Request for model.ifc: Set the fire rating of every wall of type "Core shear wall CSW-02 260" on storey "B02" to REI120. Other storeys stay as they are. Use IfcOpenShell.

First a look at what the model holds.

```python
import ifcopenshell
import ifcopenshell.util.element

model = ifcopenshell.open("model.ifc")
print(model.schema)
storey = next(s for s in model.by_type("IfcBuildingStorey") if s.Name == "B02")
walls = [e for e in ifcopenshell.util.element.get_decomposition(storey) if e.is_a("IfcWall")]
seen = {}
for e in walls:
    element_type = ifcopenshell.util.element.get_type(e)
    key = (element_type.Name if element_type != e and element_type else None, ifcopenshell.util.element.get_pset(e, "Pset_WallCommon", "FireRating"))
    seen[key] = seen.get(key, 0) + 1
for (name, value), count in sorted(seen.items(), key=str):
    print(count, "x", name, "|", value)
```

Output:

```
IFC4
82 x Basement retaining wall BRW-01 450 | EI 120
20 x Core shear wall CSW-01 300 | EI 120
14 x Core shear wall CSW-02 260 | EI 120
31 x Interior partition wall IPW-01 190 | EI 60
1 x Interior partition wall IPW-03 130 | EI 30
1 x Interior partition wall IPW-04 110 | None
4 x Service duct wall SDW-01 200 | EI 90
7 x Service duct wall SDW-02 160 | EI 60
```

```python
import ifcopenshell
import ifcopenshell.api.pset
import ifcopenshell.util.element

model = ifcopenshell.open("model.ifc")

storey = next(s for s in model.by_type("IfcBuildingStorey") if s.Name == "B02")
walls = [e for e in ifcopenshell.util.element.get_decomposition(storey) if e.is_a("IfcWall")]

count = 0
for e in walls:
    element_type = ifcopenshell.util.element.get_type(e)
    if element_type in (None, e) or element_type.Name != "Core shear wall CSW-02 260":
        continue
    # add_pset returns the element's existing set when there is one.
    pset = ifcopenshell.api.pset.add_pset(model, product=e, name="Pset_WallCommon")
    ifcopenshell.api.pset.edit_pset(model, pset=pset, properties={"FireRating": "REI120"})
    count += 1

print(count, "walls updated")

model.write("model_v2.ifc")
```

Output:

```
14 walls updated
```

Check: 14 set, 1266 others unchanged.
